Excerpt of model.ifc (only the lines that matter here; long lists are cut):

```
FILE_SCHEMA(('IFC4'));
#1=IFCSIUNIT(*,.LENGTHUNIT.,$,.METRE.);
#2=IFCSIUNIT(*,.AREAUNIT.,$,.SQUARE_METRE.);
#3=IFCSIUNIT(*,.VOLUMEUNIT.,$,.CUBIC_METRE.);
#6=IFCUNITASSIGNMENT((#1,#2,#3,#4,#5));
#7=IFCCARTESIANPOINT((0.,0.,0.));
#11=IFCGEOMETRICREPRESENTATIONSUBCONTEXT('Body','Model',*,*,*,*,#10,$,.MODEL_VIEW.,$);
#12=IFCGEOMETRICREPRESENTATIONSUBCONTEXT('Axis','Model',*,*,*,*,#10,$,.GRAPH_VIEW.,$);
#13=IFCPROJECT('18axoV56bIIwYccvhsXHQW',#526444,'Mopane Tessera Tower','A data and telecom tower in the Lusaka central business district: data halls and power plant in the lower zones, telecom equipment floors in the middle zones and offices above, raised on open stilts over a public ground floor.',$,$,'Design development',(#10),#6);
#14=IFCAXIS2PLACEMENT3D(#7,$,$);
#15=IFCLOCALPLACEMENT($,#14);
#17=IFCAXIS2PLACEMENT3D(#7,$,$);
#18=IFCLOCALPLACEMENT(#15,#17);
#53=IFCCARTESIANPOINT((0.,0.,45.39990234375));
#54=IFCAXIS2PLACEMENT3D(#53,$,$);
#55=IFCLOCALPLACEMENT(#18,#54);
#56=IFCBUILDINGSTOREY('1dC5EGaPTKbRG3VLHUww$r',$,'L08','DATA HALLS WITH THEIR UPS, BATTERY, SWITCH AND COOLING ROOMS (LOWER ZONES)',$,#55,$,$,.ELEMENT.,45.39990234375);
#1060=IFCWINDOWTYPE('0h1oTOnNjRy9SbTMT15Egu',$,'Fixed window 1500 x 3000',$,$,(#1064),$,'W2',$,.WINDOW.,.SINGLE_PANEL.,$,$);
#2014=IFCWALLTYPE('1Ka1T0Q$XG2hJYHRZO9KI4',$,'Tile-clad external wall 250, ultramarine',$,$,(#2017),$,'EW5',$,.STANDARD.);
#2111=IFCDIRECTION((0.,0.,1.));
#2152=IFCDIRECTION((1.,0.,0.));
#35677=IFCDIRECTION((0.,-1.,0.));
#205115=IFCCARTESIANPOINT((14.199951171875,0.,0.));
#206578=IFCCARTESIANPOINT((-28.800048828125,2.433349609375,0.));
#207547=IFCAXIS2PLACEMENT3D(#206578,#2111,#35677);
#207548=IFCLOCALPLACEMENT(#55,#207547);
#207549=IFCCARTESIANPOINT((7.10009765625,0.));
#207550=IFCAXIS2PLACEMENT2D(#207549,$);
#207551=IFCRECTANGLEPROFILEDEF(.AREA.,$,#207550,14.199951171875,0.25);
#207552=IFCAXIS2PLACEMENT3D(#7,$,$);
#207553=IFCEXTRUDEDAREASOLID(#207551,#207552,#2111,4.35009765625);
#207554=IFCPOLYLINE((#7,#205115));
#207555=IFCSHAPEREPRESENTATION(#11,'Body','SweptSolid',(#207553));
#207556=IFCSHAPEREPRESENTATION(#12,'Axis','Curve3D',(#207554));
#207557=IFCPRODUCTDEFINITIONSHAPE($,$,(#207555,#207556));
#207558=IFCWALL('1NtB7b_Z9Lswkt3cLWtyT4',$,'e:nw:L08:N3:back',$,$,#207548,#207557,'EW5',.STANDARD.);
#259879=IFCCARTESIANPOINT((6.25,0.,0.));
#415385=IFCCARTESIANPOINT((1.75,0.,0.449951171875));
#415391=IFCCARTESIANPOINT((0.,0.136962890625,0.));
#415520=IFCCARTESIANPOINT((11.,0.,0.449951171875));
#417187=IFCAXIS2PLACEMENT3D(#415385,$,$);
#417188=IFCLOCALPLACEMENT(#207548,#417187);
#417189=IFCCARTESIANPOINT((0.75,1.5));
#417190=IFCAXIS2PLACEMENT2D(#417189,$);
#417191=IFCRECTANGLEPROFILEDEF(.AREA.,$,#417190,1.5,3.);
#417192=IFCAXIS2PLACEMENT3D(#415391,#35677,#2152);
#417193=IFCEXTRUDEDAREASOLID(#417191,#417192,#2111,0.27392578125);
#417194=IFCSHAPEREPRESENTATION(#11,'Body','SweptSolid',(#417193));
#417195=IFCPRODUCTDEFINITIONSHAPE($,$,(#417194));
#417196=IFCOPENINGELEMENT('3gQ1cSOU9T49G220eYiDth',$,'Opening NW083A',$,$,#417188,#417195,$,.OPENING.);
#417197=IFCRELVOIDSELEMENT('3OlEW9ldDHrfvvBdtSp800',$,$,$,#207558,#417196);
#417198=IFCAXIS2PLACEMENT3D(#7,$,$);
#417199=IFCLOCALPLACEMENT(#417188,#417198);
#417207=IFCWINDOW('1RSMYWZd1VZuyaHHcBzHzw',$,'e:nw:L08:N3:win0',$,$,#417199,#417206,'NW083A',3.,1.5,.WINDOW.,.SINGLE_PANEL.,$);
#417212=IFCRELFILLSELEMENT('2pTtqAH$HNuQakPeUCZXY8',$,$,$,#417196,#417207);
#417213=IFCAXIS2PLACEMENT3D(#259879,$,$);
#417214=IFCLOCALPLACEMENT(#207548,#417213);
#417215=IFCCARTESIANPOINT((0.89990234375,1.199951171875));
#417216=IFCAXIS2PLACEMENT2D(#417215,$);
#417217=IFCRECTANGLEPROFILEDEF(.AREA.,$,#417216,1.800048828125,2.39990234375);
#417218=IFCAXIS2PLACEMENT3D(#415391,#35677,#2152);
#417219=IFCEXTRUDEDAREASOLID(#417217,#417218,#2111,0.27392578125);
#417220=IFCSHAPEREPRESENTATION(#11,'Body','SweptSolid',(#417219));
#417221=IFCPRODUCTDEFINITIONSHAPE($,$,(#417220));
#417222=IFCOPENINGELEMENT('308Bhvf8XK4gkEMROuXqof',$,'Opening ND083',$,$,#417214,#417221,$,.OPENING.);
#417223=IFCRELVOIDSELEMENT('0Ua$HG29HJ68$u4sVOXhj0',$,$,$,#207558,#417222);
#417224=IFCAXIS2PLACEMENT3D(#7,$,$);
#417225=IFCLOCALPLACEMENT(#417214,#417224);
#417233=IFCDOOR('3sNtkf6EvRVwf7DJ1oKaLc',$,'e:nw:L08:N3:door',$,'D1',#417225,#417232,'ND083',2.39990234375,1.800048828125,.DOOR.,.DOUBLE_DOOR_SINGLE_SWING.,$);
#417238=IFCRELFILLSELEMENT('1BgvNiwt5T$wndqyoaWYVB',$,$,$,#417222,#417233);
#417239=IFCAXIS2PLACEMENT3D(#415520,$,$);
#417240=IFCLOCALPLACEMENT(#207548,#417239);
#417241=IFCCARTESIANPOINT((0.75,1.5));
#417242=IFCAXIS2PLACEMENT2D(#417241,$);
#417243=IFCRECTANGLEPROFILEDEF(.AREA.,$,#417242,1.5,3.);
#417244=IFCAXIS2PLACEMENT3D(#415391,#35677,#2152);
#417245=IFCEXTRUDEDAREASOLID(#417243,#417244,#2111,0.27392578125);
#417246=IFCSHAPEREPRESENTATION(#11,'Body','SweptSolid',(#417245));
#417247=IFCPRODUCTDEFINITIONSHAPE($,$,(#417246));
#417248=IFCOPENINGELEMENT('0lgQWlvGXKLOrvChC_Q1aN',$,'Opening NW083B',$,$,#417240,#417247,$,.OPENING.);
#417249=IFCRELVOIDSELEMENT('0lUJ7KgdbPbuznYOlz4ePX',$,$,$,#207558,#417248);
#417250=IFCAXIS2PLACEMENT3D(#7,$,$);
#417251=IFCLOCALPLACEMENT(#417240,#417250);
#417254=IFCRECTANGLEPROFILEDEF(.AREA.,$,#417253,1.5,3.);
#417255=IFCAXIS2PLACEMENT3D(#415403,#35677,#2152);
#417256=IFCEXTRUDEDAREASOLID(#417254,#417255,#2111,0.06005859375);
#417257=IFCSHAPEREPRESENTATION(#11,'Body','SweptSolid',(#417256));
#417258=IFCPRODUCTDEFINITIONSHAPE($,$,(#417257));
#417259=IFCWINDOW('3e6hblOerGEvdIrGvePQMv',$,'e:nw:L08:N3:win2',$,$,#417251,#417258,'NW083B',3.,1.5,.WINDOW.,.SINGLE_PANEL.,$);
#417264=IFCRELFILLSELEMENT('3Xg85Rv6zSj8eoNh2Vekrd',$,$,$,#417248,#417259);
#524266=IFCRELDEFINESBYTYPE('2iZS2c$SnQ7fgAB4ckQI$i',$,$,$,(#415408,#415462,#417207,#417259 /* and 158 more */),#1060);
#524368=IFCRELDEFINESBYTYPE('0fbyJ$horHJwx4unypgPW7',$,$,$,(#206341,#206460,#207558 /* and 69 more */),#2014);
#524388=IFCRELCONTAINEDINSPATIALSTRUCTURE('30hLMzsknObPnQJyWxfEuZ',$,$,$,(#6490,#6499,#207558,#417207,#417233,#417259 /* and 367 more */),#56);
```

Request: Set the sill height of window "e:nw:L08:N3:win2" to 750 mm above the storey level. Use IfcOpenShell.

```python
import numpy as np
import ifcopenshell
import ifcopenshell.api.geometry
import ifcopenshell.geom
import ifcopenshell.util.element
import ifcopenshell.util.placement
import ifcopenshell.util.shape
import ifcopenshell.util.unit

model = ifcopenshell.open("model.ifc")
unit_scale = ifcopenshell.util.unit.calculate_unit_scale(model)

window = model.by_id(417259)
opening = window.FillsVoids[0].RelatingOpeningElement
storey = ifcopenshell.util.element.get_container(window, ifc_class="IfcBuildingStorey")
level = ifcopenshell.util.placement.get_local_placement(storey.ObjectPlacement)[2, 3]

# The opening's origin need not be at the sill, so measure its lowest point.
shape = ifcopenshell.geom.create_shape(ifcopenshell.geom.settings(), opening)
bottom = ifcopenshell.util.shape.get_shape_bottom_elevation(shape, shape.geometry) / unit_scale
dz = level + 0.75 / unit_scale - bottom

shift = np.array([0.0, 0.0, dz])
# The window is placed relative to its opening, so it follows when the opening moves.
matrix = ifcopenshell.util.placement.get_local_placement(opening.ObjectPlacement)
matrix[:3, 3] += shift
ifcopenshell.api.geometry.edit_object_placement(
    model, product=opening, matrix=matrix, is_si=False, should_transform_children=True
)

print(f"moved by {dz * unit_scale:+.3f} m")

model.write("model-out.ifc")
```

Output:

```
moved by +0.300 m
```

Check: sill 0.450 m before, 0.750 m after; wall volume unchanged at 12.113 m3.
